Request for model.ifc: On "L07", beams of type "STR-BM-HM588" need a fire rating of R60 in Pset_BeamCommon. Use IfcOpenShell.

First a look at what the model holds.

```python
import ifcopenshell
import ifcopenshell.util.element

model = ifcopenshell.open("model.ifc")
print(model.schema)
storey = next(s for s in model.by_type("IfcBuildingStorey") if s.Name == "L07")
beams = [e for e in ifcopenshell.util.element.get_decomposition(storey) if e.is_a("IfcBeam")]
seen = {}
for e in beams:
    element_type = ifcopenshell.util.element.get_type(e)
    key = (element_type.Name if element_type != e and element_type else None, ifcopenshell.util.element.get_pset(e, "Pset_BeamCommon", "FireRating"))
    seen[key] = seen.get(key, 0) + 1
for (name, value), count in sorted(seen.items(), key=str):
    print(count, "x", name, "|", value)
```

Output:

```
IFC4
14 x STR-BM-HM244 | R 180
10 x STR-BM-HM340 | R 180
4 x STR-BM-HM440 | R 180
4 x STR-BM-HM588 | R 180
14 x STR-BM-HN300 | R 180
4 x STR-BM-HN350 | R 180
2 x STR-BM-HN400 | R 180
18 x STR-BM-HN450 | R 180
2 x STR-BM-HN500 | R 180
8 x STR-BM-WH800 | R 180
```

```python
import ifcopenshell
import ifcopenshell.api.pset
import ifcopenshell.util.element

model = ifcopenshell.open("model.ifc")

storey = next(s for s in model.by_type("IfcBuildingStorey") if s.Name == "L07")
beams = [e for e in ifcopenshell.util.element.get_decomposition(storey) if e.is_a("IfcBeam")]

count = 0
for e in beams:
    element_type = ifcopenshell.util.element.get_type(e)
    if element_type in (None, e) or element_type.Name != "STR-BM-HM588":
        continue
    found = ifcopenshell.util.element.get_pset(e, "Pset_BeamCommon", should_inherit=False)
    if found:
        pset = model.by_id(found["id"])
        if len(ifcopenshell.util.element.get_elements_by_pset(pset)) > 1:
            pset = ifcopenshell.api.pset.unshare_pset(model, products=[e], pset=pset)[0]
    else:
        pset = ifcopenshell.api.pset.add_pset(model, product=e, name="Pset_BeamCommon")
    ifcopenshell.api.pset.edit_pset(model, pset=pset, properties={"FireRating": "R60"})
    count += 1

print(count, "beams updated")

model.write("model_updated.ifc")
```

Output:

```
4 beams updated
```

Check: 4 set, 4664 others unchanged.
